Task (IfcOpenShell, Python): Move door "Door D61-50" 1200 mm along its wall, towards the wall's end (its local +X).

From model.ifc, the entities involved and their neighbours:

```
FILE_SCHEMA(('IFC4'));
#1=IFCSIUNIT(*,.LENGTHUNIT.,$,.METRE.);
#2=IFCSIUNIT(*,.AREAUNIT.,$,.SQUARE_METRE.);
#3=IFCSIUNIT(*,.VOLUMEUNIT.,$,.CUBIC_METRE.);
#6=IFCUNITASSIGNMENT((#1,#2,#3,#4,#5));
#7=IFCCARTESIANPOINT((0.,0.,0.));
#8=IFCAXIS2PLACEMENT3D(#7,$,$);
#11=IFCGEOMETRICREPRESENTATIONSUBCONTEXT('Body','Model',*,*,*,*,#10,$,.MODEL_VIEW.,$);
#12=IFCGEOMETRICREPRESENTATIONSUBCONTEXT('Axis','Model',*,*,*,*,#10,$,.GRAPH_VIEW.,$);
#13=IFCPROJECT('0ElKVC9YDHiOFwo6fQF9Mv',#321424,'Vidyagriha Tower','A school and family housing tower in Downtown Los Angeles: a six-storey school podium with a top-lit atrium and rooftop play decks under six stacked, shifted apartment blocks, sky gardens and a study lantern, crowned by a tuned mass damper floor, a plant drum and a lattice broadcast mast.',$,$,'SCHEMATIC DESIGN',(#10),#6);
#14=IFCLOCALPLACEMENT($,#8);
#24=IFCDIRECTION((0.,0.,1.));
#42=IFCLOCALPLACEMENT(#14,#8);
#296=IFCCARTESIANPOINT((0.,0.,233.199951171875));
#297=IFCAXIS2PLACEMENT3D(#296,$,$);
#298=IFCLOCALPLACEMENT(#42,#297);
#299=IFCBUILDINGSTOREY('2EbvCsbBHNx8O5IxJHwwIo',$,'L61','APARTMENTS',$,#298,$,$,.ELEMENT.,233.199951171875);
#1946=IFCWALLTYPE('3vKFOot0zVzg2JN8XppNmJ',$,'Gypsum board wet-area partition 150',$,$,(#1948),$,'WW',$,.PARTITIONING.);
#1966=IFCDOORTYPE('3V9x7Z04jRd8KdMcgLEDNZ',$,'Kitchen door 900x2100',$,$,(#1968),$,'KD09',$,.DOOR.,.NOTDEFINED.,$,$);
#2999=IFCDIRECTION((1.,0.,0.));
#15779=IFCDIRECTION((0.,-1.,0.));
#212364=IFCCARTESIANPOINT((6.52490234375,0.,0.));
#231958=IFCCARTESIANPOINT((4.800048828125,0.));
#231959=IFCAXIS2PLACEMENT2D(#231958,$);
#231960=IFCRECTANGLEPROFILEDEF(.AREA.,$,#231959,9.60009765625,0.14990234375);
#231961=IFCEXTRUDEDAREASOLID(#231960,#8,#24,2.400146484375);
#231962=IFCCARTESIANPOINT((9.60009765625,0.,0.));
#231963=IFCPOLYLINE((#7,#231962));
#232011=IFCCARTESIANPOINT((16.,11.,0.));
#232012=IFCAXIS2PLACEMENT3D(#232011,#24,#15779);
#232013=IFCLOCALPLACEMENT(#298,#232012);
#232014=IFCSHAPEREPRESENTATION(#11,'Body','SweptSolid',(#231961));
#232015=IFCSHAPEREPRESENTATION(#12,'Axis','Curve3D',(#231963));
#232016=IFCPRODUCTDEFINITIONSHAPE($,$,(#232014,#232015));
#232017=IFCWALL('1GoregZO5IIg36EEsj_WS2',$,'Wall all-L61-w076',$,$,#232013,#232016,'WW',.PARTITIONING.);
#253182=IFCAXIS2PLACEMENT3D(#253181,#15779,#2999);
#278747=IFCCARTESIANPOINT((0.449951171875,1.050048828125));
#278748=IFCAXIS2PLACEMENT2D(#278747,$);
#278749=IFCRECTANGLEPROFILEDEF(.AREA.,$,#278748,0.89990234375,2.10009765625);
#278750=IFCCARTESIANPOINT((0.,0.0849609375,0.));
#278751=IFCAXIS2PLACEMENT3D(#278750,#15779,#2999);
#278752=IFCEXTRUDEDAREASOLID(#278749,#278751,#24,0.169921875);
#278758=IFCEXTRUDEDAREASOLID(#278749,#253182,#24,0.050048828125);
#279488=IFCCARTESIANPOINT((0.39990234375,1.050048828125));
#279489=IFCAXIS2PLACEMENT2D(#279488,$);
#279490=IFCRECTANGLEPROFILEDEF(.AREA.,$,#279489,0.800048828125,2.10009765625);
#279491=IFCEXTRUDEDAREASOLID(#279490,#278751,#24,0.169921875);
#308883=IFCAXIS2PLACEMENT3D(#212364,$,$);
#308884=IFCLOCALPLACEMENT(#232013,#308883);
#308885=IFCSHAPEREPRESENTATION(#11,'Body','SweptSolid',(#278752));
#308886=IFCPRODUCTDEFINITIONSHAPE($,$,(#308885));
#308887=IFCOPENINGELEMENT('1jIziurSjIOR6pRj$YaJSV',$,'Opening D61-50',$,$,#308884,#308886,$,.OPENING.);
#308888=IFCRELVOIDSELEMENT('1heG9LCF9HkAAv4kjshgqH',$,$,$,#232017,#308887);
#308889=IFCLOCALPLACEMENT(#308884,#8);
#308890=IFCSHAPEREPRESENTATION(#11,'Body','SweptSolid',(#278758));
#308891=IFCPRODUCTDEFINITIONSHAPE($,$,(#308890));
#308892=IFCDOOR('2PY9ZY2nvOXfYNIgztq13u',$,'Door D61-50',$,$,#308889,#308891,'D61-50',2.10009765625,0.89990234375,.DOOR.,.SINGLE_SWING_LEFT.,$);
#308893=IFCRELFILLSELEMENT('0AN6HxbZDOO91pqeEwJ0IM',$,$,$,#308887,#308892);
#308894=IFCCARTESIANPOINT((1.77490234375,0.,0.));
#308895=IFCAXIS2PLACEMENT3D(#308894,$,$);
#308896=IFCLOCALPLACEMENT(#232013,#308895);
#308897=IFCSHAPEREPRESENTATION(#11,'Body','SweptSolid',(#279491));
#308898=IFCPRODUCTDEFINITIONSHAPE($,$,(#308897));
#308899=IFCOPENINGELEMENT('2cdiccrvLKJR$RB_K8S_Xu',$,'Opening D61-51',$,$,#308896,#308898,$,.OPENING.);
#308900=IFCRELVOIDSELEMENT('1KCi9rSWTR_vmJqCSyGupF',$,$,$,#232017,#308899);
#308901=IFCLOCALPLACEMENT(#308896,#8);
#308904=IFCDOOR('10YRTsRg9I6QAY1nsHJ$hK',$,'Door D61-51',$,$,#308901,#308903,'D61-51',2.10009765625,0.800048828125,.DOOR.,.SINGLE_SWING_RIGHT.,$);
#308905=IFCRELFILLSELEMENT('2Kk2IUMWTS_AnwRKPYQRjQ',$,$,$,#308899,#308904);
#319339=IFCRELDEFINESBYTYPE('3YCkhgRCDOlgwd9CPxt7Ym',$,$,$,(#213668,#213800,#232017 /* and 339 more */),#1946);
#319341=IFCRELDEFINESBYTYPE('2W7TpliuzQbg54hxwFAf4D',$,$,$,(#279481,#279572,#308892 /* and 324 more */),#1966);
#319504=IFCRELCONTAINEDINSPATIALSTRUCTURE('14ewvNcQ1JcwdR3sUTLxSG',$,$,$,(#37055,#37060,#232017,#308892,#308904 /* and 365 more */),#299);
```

```python
import ifcopenshell
import ifcopenshell.api.geometry
import ifcopenshell.util.placement
import ifcopenshell.util.unit

model = ifcopenshell.open("model.ifc")
unit_scale = ifcopenshell.util.unit.calculate_unit_scale(model)

door = model.by_id(308892)
opening = door.FillsVoids[0].RelatingOpeningElement
wall = opening.VoidsElements[0].RelatingBuildingElement

wall_matrix = ifcopenshell.util.placement.get_local_placement(wall.ObjectPlacement)
shift = wall_matrix[:3, 0] * 1.2 / unit_scale
before = ifcopenshell.util.placement.get_local_placement(door.ObjectPlacement)[:3, 3].copy()

# The door is placed relative to its opening, so it follows when the opening moves.
matrix = ifcopenshell.util.placement.get_local_placement(opening.ObjectPlacement)
matrix[:3, 3] += shift
ifcopenshell.api.geometry.edit_object_placement(
    model, product=opening, matrix=matrix, is_si=False, should_transform_children=True
)

after = ifcopenshell.util.placement.get_local_placement(door.ObjectPlacement)[:3, 3]
print("door moved by", (after - before).round(3) + 0.0)

model.write("model_rev.ifc")
```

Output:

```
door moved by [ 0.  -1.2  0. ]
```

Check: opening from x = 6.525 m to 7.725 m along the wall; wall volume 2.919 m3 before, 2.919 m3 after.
